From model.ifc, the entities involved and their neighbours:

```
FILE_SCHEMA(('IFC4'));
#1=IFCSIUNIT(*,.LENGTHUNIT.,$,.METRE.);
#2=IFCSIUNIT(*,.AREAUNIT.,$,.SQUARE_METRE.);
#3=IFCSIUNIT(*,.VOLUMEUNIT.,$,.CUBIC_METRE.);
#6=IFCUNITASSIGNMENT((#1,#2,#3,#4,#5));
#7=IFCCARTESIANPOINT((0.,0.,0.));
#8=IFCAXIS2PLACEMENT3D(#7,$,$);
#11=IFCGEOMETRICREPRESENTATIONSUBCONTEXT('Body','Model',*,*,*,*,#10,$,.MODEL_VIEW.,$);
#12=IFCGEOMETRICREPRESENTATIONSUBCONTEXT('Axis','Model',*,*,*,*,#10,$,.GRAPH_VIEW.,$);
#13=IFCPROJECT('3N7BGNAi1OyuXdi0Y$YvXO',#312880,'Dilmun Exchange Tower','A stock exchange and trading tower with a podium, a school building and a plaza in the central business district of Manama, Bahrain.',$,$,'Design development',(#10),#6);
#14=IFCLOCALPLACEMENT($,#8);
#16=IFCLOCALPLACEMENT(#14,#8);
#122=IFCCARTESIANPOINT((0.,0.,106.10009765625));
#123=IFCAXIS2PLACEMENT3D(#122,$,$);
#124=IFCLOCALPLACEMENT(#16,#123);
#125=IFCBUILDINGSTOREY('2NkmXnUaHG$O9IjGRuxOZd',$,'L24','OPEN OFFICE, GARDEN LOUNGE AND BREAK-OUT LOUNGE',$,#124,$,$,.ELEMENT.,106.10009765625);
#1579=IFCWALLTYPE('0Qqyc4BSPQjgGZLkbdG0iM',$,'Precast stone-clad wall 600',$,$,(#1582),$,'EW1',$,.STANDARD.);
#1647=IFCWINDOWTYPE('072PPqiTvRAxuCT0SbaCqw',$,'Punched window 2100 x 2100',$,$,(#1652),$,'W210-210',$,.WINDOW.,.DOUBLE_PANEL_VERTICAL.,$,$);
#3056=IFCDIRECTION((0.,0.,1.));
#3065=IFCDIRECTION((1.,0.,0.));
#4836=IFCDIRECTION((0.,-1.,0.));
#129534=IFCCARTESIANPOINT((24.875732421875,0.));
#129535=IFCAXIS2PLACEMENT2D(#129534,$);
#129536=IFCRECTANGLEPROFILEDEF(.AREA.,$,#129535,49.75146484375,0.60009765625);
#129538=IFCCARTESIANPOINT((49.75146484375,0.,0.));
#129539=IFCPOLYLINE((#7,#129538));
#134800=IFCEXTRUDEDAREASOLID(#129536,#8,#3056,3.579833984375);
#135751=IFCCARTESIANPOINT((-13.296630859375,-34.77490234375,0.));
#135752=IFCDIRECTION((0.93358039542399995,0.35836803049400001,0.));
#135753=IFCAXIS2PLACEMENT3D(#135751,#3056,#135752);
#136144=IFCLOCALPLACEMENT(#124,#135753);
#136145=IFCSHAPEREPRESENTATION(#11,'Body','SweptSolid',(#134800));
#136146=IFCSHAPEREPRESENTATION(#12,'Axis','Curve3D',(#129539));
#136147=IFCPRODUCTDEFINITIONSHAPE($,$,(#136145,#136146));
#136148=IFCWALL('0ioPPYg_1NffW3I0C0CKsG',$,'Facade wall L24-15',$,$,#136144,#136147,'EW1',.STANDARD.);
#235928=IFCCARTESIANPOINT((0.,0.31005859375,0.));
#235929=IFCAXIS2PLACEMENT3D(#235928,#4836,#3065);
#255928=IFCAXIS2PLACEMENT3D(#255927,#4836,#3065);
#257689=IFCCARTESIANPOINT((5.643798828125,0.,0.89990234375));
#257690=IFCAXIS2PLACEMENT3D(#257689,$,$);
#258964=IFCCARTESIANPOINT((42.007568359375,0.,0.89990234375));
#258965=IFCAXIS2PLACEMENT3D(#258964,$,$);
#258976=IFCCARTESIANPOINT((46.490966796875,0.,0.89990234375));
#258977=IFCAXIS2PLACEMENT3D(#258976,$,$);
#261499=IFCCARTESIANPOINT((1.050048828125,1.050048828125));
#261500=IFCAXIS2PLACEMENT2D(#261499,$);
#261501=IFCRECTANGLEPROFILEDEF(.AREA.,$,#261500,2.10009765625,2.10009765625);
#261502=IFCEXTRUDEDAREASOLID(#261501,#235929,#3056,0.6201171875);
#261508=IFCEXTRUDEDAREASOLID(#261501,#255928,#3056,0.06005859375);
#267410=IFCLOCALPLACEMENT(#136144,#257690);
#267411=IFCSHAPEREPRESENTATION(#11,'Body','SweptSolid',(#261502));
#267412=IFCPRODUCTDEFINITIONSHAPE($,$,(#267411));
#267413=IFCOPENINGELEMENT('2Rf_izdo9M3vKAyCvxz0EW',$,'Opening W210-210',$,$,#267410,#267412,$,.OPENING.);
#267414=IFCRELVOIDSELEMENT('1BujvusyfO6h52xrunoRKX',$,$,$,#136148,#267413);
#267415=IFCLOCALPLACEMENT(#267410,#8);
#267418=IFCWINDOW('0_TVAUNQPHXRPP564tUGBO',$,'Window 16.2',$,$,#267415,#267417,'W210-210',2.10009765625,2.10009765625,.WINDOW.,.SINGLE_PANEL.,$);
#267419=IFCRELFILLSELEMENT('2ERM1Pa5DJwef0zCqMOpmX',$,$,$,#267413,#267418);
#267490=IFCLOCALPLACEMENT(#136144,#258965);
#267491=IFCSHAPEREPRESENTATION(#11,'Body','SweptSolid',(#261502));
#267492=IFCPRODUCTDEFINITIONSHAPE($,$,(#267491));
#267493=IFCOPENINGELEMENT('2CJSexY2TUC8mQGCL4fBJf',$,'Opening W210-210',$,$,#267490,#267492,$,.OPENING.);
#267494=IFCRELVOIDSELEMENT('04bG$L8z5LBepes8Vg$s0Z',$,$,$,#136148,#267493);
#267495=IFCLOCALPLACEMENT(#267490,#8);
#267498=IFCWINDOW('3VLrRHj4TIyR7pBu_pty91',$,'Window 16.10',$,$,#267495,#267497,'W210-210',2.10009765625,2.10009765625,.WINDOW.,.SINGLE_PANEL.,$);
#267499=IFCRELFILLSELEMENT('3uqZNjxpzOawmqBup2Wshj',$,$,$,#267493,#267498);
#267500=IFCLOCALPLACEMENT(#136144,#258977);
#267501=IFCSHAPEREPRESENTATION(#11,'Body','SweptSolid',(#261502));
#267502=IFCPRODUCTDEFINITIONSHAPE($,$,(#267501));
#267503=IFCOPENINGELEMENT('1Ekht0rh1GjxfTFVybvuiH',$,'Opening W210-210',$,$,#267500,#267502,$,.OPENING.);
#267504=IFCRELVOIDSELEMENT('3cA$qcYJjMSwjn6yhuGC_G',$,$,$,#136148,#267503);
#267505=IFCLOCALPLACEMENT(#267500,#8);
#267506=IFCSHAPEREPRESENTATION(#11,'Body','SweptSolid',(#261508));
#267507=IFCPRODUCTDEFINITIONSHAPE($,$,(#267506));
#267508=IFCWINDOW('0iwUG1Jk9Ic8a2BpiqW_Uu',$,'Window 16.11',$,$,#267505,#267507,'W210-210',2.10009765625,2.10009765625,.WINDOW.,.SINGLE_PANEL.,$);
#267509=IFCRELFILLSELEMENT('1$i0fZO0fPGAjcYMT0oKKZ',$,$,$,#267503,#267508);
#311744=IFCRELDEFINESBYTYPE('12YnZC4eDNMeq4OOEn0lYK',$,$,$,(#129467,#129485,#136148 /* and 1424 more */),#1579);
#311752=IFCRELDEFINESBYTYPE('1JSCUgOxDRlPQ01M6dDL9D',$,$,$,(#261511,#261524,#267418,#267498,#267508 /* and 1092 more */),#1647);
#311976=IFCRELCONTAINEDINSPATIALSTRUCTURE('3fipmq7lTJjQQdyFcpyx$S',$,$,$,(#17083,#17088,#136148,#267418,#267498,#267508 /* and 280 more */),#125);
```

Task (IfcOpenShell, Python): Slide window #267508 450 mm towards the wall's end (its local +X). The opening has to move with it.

```python
import ifcopenshell
import ifcopenshell.api.geometry
import ifcopenshell.util.placement

model = ifcopenshell.open("model.ifc")

window = model.by_id(267508)
opening = window.FillsVoids[0].RelatingOpeningElement
wall = opening.VoidsElements[0].RelatingBuildingElement

wall_matrix = ifcopenshell.util.placement.get_local_placement(wall.ObjectPlacement)
shift = wall_matrix[:3, 0] * 0.45
before = ifcopenshell.util.placement.get_local_placement(window.ObjectPlacement)[:3, 3].copy()

# The window is placed relative to its opening, so it follows when the opening moves.
matrix = ifcopenshell.util.placement.get_local_placement(opening.ObjectPlacement)
matrix[:3, 3] += shift
ifcopenshell.api.geometry.edit_object_placement(
    model, product=opening, matrix=matrix, is_si=False, should_transform_children=True
)

after = ifcopenshell.util.placement.get_local_placement(window.ObjectPlacement)[:3, 3]
print("window moved by", (after - before).round(3) + 0.0)

model.write("model_rev.ifc")
```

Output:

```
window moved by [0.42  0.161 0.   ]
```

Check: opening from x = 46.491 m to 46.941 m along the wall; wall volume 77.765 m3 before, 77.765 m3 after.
